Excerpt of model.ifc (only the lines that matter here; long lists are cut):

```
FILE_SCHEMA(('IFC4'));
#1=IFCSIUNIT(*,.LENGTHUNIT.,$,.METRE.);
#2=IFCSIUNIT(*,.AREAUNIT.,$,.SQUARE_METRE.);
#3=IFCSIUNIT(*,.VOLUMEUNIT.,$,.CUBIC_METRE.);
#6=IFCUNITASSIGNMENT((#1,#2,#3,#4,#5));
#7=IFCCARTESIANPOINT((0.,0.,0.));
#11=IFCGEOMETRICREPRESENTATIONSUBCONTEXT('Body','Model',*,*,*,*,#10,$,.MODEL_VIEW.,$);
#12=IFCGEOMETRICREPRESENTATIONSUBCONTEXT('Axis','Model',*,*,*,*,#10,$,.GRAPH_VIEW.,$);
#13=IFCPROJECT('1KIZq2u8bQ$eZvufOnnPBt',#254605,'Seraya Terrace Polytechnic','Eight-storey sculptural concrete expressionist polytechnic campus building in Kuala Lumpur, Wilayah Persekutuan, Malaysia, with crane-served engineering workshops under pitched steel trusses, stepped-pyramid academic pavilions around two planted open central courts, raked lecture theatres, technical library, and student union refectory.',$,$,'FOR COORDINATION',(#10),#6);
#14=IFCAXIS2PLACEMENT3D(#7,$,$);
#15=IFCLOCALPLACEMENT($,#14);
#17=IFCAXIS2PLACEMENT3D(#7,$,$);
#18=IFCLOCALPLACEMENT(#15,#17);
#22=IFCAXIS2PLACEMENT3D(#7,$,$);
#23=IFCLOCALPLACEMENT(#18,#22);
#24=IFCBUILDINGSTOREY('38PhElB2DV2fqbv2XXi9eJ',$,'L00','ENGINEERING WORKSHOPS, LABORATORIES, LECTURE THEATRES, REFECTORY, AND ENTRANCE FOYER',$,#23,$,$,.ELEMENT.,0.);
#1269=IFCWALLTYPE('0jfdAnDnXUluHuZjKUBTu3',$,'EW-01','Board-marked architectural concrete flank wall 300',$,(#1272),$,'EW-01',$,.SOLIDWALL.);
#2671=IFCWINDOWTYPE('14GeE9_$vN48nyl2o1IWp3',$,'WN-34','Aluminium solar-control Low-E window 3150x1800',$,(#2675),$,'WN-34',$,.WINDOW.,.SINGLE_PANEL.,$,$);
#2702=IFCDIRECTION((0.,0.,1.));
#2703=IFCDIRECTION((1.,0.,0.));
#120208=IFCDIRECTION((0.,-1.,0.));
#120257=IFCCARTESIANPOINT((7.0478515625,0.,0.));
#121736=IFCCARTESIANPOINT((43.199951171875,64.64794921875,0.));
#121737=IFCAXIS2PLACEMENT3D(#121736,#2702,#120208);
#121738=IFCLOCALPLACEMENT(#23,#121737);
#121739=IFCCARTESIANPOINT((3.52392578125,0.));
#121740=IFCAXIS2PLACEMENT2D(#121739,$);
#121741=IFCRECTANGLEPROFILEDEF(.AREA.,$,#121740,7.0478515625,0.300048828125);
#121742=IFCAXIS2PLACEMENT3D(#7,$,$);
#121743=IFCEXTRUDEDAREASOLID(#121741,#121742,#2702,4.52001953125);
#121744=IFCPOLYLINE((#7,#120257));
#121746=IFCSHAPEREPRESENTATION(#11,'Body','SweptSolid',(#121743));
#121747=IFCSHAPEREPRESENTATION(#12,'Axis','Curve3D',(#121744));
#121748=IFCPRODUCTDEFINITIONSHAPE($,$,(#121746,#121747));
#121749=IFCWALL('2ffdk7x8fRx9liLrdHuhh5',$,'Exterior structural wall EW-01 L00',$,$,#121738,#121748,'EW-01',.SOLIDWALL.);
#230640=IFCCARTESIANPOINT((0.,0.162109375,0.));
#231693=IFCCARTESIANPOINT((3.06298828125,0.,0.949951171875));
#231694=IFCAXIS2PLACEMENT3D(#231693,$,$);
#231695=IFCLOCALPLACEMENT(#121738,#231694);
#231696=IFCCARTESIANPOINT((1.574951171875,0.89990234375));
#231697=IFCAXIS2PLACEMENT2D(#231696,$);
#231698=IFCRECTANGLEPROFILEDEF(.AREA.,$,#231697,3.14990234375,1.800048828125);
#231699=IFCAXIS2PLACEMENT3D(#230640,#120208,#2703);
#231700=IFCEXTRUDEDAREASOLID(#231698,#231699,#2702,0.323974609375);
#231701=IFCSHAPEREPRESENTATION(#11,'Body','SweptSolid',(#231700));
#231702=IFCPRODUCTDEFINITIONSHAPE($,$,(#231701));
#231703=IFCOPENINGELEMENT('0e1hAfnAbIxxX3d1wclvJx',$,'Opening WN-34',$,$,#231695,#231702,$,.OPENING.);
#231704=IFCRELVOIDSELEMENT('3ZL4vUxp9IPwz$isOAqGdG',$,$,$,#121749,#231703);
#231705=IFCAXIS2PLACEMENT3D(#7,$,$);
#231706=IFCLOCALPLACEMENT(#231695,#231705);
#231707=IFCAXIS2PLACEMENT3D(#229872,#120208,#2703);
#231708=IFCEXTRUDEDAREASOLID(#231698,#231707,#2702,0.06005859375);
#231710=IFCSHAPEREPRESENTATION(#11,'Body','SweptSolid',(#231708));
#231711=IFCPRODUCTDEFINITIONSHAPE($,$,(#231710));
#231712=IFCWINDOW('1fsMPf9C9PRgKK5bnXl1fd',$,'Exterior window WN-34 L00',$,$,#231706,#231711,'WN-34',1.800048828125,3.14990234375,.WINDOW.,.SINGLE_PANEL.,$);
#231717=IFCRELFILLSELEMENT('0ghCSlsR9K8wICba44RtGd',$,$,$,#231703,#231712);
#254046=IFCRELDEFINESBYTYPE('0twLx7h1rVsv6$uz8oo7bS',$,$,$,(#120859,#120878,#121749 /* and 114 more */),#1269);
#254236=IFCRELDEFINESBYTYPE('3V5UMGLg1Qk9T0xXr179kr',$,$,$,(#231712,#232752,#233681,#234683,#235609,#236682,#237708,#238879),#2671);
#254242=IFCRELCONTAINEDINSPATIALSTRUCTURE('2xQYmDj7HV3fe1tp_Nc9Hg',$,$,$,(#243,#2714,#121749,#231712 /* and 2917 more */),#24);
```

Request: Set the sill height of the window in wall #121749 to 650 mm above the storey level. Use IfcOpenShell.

```python
import numpy as np
import ifcopenshell
import ifcopenshell.api.geometry
import ifcopenshell.geom
import ifcopenshell.util.element
import ifcopenshell.util.placement
import ifcopenshell.util.shape
import ifcopenshell.util.unit

model = ifcopenshell.open("model.ifc")
unit_scale = ifcopenshell.util.unit.calculate_unit_scale(model)

window = model.by_guid("1fsMPf9C9PRgKK5bnXl1fd")
opening = window.FillsVoids[0].RelatingOpeningElement
storey = ifcopenshell.util.element.get_container(window, ifc_class="IfcBuildingStorey")
level = ifcopenshell.util.placement.get_local_placement(storey.ObjectPlacement)[2, 3]

# The opening's origin need not be at the sill, so measure its lowest point.
shape = ifcopenshell.geom.create_shape(ifcopenshell.geom.settings(), opening)
bottom = ifcopenshell.util.shape.get_shape_bottom_elevation(shape, shape.geometry) / unit_scale
dz = level + 0.65 / unit_scale - bottom

shift = np.array([0.0, 0.0, dz])
# The window is placed relative to its opening, so it follows when the opening moves.
matrix = ifcopenshell.util.placement.get_local_placement(opening.ObjectPlacement)
matrix[:3, 3] += shift
ifcopenshell.api.geometry.edit_object_placement(
    model, product=opening, matrix=matrix, is_si=False, should_transform_children=True
)

print(f"moved by {dz * unit_scale:+.3f} m")

model.write("model-out.ifc")
```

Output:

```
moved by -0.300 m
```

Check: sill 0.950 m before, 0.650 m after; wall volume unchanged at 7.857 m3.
